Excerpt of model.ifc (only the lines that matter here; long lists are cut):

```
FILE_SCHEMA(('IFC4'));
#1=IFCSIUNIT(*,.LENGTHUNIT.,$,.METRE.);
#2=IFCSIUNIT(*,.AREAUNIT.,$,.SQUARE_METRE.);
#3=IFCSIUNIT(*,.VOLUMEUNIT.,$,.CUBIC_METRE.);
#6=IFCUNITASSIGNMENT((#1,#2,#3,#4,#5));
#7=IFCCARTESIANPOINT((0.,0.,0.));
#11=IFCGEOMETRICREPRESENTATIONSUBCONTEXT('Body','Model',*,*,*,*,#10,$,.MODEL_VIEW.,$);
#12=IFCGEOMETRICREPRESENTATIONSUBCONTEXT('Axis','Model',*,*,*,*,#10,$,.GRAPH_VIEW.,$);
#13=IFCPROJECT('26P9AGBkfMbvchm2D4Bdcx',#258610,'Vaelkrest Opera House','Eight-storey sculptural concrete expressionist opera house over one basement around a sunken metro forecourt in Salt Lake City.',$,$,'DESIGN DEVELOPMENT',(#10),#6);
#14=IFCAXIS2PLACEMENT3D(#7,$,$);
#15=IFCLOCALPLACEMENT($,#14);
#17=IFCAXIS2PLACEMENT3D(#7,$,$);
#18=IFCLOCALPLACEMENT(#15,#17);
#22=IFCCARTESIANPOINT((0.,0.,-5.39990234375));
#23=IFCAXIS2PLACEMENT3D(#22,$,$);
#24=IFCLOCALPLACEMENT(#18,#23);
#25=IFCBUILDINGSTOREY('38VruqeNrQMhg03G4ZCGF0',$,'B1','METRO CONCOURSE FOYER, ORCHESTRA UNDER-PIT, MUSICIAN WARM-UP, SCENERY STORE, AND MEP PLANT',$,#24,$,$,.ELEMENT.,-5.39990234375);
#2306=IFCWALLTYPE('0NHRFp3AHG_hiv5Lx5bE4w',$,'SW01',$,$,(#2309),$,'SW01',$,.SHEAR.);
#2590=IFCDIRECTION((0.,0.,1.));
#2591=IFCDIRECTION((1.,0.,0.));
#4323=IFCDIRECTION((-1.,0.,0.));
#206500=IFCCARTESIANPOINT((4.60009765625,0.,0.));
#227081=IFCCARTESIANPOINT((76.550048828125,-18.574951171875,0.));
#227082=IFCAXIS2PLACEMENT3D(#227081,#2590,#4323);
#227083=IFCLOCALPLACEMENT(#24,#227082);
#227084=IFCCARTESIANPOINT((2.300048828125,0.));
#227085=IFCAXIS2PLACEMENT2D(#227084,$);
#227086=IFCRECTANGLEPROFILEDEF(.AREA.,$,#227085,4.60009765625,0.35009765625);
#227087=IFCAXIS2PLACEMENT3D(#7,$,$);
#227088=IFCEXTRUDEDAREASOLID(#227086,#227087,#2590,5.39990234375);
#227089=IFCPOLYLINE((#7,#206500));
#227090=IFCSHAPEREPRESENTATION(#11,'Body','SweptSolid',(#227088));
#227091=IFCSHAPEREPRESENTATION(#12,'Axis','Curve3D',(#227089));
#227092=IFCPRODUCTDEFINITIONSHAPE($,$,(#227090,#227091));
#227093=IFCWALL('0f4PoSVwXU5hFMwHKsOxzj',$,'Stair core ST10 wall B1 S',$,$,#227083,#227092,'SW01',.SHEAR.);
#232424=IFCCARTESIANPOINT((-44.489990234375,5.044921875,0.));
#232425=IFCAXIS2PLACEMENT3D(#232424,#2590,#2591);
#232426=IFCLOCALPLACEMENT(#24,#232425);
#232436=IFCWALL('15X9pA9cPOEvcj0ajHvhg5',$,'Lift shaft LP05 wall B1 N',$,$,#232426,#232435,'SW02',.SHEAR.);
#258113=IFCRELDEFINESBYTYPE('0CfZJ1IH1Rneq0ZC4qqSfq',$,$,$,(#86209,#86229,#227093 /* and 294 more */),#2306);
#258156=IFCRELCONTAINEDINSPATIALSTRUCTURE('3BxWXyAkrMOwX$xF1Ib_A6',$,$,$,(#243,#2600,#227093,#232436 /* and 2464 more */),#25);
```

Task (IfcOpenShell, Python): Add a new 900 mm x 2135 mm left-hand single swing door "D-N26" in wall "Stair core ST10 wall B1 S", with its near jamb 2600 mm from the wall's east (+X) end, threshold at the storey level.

```python
import numpy as np
import ifcopenshell
import ifcopenshell.api.feature
import ifcopenshell.api.geometry
import ifcopenshell.api.root
import ifcopenshell.api.spatial
import ifcopenshell.geom
import ifcopenshell.util.element
import ifcopenshell.util.placement
import ifcopenshell.util.representation
import ifcopenshell.util.shape
import ifcopenshell.util.unit

model = ifcopenshell.open("model.ifc")
unit_scale = ifcopenshell.util.unit.calculate_unit_scale(model)
settings = ifcopenshell.geom.settings()


def volume(element):
    """Net volume in cubic metres, openings subtracted."""
    shape = ifcopenshell.geom.create_shape(settings, element)
    return ifcopenshell.util.shape.get_volume(shape.geometry)


wall = model.by_guid("0f4PoSVwXU5hFMwHKsOxzj")
storey = ifcopenshell.util.element.get_container(wall, ifc_class="IfcBuildingStorey")
context = ifcopenshell.util.representation.get_context(model, "Model", "Body", "MODEL_VIEW")
before = volume(wall)

width, height, from_end, sill = 0.9, 2.135, 2.6, 0.0  # metres

# The wall runs along its own X axis, and the end named is its -X end.
wall_shape = ifcopenshell.geom.create_shape(settings, wall)
x, y, z = ifcopenshell.util.shape.get_vertices(wall_shape.geometry).T
start = x.min() + from_end
face, thickness = float(y.min()), float(y.max() - y.min())
wall_matrix = ifcopenshell.util.placement.get_local_placement(wall.ObjectPlacement)
level = ifcopenshell.util.placement.get_local_placement(storey.ObjectPlacement)[2, 3]


def in_wall(x, y):
    """Placement at x, y metres in the wall's axes, at sill height."""
    matrix = wall_matrix.copy()
    matrix[:, 3] = wall_matrix @ np.array([x / unit_scale, y / unit_scale, 0.0, 1.0])
    matrix[2, 3] = level + sill / unit_scale
    return matrix


# Opening: a box that overshoots both wall faces by 50 mm.
opening = ifcopenshell.api.root.create_entity(model, ifc_class="IfcOpeningElement", predefined_type="OPENING")
box = ifcopenshell.api.geometry.add_wall_representation(
    model, context=context, length=width, height=height, thickness=thickness + 0.1
)
ifcopenshell.api.geometry.assign_representation(model, product=opening, representation=box)
ifcopenshell.api.geometry.edit_object_placement(model, product=opening, matrix=in_wall(start, face - 0.05), is_si=False)
ifcopenshell.api.feature.add_feature(model, feature=opening, element=wall)

door = ifcopenshell.api.root.create_entity(model, ifc_class="IfcDoor", name="D-N26", predefined_type="DOOR")
door.OverallWidth, door.OverallHeight = width / unit_scale, height / unit_scale
door.OperationType = "SINGLE_SWING_LEFT"
body = ifcopenshell.api.geometry.add_door_representation(
    model,
    context=context,
    overall_width=door.OverallWidth,
    overall_height=door.OverallHeight,
    operation_type="SINGLE_SWING_LEFT",
    lining_properties={"LiningDepth": thickness / unit_scale, "ThresholdDepth": thickness / unit_scale},
)
ifcopenshell.api.geometry.assign_representation(model, product=door, representation=body)
ifcopenshell.api.spatial.assign_container(model, products=[door], relating_structure=storey)
ifcopenshell.api.feature.add_filling(model, opening=opening, element=door)

# The lining spans the wall, so the door starts at the wall face.
ifcopenshell.api.geometry.edit_object_placement(model, product=door, matrix=in_wall(start, face), is_si=False)

after = volume(wall)

print(f"wall volume {before:.3f} -> {after:.3f} m3")

model.write("model_edited.ifc")
```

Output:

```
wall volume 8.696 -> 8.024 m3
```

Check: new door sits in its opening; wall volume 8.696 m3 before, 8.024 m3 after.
